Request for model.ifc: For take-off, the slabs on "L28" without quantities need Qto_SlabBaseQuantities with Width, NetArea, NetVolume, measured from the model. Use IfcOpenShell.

First a look at what the model holds.

```python
import ifcopenshell
import ifcopenshell.util.element
import ifcopenshell.util.unit

model = ifcopenshell.open("model.ifc")
print(model.schema)
for unit_type in ("LENGTHUNIT", "AREAUNIT", "VOLUMEUNIT"):
    print(unit_type, ifcopenshell.util.unit.calculate_unit_scale(model, unit_type))
storey = next(s for s in model.by_type("IfcBuildingStorey") if s.Name == "L28")
slabs = [e for e in ifcopenshell.util.element.get_decomposition(storey) if e.is_a("IfcSlab")]
for e in sorted(slabs, key=lambda e: e.id()):
    print(e.id(), e.is_a(), e.Name, list(ifcopenshell.util.element.get_psets(e, qtos_only=True)), sep=" | ")
```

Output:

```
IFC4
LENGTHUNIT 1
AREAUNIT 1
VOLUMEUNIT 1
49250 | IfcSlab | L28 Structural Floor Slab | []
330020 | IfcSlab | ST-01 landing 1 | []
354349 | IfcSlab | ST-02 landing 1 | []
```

```python
import ifcopenshell
import ifcopenshell.api.pset
import ifcopenshell.geom
import ifcopenshell.util.element
import ifcopenshell.util.shape
import ifcopenshell.util.unit

model = ifcopenshell.open("model.ifc")
unit_scale = ifcopenshell.util.unit.calculate_unit_scale(model)
area_scale = ifcopenshell.util.unit.calculate_unit_scale(model, "AREAUNIT")
volume_scale = ifcopenshell.util.unit.calculate_unit_scale(model, "VOLUMEUNIT")
settings = ifcopenshell.geom.settings()

storey = next(s for s in model.by_type("IfcBuildingStorey") if s.Name == "L28")
slabs = [e for e in ifcopenshell.util.element.get_decomposition(storey) if e.is_a("IfcSlab")]

for e in sorted(slabs, key=lambda e: e.id()):
    if ifcopenshell.util.element.get_psets(e, qtos_only=True, should_inherit=False):
        continue
    # Geometry comes back in metres, in the element's own axes.
    shape = ifcopenshell.geom.create_shape(settings, e)
    values = {
        "Width": ifcopenshell.util.shape.get_z(shape.geometry) / unit_scale,
        "NetArea": ifcopenshell.util.shape.get_footprint_area(shape.geometry) / area_scale,
        "NetVolume": ifcopenshell.util.shape.get_volume(shape.geometry) / volume_scale,
    }
    qto = ifcopenshell.api.pset.add_qto(model, product=e, name="Qto_SlabBaseQuantities")
    ifcopenshell.api.pset.edit_qto(model, qto=qto, properties=values)
    print(e.id(), {k: round(v, 3) for k, v in values.items()})

model.write("model_updated.ifc")
```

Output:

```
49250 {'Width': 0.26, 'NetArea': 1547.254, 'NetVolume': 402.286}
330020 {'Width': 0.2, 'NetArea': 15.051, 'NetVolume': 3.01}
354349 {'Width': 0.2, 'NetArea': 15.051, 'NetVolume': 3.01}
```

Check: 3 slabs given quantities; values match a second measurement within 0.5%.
